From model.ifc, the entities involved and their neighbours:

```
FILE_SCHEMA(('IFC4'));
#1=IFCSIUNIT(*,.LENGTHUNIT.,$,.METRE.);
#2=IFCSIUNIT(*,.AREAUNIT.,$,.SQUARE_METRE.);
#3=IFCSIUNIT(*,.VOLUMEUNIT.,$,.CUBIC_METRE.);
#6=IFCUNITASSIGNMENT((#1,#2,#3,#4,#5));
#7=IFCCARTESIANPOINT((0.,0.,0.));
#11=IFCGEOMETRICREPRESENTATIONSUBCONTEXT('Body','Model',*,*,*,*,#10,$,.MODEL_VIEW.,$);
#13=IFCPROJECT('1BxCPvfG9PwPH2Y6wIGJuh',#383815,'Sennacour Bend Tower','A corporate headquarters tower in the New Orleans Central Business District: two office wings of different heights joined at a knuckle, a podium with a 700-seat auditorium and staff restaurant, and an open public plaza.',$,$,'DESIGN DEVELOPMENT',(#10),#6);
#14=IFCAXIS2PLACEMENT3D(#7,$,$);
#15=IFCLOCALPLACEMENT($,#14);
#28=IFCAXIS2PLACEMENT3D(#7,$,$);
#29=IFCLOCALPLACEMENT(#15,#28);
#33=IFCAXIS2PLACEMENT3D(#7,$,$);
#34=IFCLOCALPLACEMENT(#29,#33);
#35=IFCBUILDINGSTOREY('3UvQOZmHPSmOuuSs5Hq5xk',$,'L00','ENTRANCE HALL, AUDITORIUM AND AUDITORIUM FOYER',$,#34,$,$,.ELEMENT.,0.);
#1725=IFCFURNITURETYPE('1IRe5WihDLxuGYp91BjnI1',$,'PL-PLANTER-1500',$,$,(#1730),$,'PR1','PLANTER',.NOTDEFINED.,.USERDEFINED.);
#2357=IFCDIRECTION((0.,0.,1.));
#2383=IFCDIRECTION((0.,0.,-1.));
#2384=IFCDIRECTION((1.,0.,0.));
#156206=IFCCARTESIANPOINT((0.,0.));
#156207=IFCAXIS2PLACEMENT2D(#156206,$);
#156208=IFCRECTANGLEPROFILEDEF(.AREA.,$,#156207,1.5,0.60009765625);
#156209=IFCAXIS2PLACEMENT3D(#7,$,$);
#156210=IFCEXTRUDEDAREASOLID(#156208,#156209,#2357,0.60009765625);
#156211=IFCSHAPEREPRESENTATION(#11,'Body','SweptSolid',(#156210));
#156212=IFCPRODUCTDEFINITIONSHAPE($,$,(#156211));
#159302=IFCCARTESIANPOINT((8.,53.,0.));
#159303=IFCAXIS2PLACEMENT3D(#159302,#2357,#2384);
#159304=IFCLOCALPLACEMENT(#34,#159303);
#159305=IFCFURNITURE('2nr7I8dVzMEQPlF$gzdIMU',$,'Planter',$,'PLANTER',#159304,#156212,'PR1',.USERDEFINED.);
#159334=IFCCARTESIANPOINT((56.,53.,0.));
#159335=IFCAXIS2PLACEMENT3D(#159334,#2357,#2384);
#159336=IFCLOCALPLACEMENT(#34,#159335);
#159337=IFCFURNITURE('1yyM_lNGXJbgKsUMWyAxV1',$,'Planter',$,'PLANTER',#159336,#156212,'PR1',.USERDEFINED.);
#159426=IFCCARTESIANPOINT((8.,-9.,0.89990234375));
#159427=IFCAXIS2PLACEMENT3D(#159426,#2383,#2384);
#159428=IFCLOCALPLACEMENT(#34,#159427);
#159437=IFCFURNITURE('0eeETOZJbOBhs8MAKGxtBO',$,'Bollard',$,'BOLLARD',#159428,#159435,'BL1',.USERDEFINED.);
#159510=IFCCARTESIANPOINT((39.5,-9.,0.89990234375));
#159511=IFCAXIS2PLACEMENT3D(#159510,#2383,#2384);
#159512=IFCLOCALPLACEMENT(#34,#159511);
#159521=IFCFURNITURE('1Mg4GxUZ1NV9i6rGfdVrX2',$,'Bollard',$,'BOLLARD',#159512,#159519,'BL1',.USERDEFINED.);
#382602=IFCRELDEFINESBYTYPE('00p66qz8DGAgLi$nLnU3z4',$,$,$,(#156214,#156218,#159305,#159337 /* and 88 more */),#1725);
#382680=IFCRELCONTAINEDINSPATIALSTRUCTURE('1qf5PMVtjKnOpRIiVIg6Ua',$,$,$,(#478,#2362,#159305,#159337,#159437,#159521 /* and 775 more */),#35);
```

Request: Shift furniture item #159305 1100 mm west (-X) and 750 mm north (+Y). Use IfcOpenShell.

```python
import ifcopenshell
import ifcopenshell.api.geometry
import ifcopenshell.util.placement
import ifcopenshell.util.unit

model = ifcopenshell.open("model.ifc")
unit_scale = ifcopenshell.util.unit.calculate_unit_scale(model)

item = model.by_guid("2nr7I8dVzMEQPlF$gzdIMU")
matrix = ifcopenshell.util.placement.get_local_placement(item.ObjectPlacement)
matrix[0, 3] -= 1.1 / unit_scale
matrix[1, 3] += 0.75 / unit_scale
ifcopenshell.api.geometry.edit_object_placement(model, product=item, matrix=matrix, is_si=False)

print(ifcopenshell.util.placement.get_local_placement(item.ObjectPlacement).round(3) + 0.0)

model.write("model_v2.ifc")
```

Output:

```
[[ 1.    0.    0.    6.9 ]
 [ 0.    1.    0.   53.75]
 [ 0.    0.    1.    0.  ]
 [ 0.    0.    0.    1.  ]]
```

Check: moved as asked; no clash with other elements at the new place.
